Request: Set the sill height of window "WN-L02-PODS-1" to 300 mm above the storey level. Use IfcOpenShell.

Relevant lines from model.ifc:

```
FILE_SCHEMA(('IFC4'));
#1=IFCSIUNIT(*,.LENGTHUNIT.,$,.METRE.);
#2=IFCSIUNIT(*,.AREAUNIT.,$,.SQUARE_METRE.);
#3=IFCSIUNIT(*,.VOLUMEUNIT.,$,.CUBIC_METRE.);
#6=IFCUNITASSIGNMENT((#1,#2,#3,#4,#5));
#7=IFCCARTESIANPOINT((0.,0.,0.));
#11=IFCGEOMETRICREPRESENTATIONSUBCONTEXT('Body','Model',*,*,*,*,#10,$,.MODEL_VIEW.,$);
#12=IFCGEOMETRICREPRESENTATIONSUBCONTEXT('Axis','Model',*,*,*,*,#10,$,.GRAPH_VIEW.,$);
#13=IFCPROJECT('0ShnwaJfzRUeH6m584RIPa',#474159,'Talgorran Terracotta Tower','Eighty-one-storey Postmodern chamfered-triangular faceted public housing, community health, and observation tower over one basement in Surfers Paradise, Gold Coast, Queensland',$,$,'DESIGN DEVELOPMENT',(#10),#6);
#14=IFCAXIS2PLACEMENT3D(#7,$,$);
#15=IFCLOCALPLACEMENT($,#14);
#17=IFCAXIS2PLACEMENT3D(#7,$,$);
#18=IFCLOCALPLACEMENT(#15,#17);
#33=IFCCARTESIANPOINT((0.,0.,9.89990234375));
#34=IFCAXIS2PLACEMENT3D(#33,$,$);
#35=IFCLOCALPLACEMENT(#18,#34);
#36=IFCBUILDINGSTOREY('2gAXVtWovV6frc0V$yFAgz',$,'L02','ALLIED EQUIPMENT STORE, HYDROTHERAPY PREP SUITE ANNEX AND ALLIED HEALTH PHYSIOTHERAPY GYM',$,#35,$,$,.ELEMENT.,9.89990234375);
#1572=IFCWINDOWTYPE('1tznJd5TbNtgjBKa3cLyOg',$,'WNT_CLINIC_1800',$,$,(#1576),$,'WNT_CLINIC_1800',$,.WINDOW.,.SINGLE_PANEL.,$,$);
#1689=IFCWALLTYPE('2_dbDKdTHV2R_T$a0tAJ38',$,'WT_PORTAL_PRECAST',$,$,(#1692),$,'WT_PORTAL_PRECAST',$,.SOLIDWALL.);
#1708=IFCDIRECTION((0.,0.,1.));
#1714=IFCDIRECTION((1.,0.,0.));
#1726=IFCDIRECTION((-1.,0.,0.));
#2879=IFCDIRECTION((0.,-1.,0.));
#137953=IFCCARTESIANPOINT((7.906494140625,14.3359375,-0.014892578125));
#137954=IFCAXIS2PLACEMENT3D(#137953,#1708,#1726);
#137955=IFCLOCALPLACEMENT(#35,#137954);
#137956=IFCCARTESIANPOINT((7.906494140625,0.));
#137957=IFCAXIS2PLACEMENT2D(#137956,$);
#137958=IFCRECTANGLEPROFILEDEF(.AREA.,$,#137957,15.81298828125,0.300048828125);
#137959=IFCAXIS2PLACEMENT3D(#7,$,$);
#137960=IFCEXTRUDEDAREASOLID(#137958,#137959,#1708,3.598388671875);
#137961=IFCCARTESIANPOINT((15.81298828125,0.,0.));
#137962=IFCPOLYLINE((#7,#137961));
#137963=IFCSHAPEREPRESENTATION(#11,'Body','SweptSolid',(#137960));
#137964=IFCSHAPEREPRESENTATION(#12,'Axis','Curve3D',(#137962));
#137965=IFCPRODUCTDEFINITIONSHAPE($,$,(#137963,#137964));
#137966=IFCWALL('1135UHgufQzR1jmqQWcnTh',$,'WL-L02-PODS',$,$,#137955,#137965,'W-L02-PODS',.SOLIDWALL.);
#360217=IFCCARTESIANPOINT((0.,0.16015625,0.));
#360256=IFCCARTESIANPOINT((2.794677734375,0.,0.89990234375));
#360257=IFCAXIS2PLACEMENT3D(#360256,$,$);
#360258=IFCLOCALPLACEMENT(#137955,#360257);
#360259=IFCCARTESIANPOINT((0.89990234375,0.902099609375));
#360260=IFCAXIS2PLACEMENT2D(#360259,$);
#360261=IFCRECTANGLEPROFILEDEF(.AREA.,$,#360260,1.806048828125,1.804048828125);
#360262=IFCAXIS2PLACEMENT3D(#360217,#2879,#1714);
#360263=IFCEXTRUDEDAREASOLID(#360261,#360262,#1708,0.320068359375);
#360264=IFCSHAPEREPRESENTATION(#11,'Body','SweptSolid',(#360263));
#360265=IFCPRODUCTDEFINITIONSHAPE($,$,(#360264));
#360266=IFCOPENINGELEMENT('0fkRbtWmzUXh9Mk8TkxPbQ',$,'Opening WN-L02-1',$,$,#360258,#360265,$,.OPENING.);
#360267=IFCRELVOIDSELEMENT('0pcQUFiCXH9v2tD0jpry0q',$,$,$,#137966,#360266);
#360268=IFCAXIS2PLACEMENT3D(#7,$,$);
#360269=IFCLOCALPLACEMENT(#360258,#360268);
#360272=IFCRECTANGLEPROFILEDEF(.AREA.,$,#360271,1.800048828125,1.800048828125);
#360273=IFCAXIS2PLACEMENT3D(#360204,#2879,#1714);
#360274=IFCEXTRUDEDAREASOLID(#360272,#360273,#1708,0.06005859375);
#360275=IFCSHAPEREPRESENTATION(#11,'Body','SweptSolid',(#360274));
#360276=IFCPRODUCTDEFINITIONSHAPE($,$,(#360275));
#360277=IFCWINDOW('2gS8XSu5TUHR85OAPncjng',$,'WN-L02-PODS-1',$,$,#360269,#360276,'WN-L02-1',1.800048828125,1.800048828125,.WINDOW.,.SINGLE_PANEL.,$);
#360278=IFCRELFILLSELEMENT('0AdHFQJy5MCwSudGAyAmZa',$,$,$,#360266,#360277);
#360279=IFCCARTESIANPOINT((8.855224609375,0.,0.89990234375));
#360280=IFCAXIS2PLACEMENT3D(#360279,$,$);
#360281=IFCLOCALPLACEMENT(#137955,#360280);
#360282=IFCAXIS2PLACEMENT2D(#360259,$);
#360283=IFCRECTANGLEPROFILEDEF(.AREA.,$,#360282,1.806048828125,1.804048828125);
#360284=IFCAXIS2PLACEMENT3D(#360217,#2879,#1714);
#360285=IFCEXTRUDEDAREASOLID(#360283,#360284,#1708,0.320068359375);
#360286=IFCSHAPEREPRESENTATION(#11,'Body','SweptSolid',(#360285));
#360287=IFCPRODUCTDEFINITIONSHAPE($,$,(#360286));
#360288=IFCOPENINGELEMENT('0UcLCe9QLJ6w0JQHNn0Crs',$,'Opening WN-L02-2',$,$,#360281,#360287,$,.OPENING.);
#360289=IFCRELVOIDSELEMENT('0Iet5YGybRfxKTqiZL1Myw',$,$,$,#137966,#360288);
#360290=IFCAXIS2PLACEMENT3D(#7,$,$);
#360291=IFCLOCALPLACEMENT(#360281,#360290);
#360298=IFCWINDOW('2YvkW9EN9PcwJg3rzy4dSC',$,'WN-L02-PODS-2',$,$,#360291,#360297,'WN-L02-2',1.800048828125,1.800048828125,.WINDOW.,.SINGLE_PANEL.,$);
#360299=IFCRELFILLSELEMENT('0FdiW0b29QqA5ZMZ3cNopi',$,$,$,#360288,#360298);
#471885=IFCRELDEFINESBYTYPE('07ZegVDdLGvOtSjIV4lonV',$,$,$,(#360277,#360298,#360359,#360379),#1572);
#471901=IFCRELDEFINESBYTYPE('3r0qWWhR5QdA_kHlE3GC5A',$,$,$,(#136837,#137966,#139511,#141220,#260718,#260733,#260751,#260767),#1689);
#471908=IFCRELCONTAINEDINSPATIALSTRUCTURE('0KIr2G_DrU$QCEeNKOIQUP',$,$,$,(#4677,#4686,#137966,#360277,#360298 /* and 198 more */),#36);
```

```python
import numpy as np
import ifcopenshell
import ifcopenshell.api.geometry
import ifcopenshell.geom
import ifcopenshell.util.element
import ifcopenshell.util.placement
import ifcopenshell.util.shape
import ifcopenshell.util.unit

model = ifcopenshell.open("model.ifc")
unit_scale = ifcopenshell.util.unit.calculate_unit_scale(model)

window = model.by_guid("2gS8XSu5TUHR85OAPncjng")
opening = window.FillsVoids[0].RelatingOpeningElement
storey = ifcopenshell.util.element.get_container(window, ifc_class="IfcBuildingStorey")
level = ifcopenshell.util.placement.get_local_placement(storey.ObjectPlacement)[2, 3]

# The opening's origin need not be at the sill, so measure its lowest point.
shape = ifcopenshell.geom.create_shape(ifcopenshell.geom.settings(), opening)
bottom = ifcopenshell.util.shape.get_shape_bottom_elevation(shape, shape.geometry) / unit_scale
dz = level + 0.3 / unit_scale - bottom

shift = np.array([0.0, 0.0, dz])
# The window is placed relative to its opening, so it follows when the opening moves.
matrix = ifcopenshell.util.placement.get_local_placement(opening.ObjectPlacement)
matrix[:3, 3] += shift
ifcopenshell.api.geometry.edit_object_placement(
    model, product=opening, matrix=matrix, is_si=False, should_transform_children=True
)

print(f"moved by {dz * unit_scale:+.3f} m")

model.write("model-out.ifc")
```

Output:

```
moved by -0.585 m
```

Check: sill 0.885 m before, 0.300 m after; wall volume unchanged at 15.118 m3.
